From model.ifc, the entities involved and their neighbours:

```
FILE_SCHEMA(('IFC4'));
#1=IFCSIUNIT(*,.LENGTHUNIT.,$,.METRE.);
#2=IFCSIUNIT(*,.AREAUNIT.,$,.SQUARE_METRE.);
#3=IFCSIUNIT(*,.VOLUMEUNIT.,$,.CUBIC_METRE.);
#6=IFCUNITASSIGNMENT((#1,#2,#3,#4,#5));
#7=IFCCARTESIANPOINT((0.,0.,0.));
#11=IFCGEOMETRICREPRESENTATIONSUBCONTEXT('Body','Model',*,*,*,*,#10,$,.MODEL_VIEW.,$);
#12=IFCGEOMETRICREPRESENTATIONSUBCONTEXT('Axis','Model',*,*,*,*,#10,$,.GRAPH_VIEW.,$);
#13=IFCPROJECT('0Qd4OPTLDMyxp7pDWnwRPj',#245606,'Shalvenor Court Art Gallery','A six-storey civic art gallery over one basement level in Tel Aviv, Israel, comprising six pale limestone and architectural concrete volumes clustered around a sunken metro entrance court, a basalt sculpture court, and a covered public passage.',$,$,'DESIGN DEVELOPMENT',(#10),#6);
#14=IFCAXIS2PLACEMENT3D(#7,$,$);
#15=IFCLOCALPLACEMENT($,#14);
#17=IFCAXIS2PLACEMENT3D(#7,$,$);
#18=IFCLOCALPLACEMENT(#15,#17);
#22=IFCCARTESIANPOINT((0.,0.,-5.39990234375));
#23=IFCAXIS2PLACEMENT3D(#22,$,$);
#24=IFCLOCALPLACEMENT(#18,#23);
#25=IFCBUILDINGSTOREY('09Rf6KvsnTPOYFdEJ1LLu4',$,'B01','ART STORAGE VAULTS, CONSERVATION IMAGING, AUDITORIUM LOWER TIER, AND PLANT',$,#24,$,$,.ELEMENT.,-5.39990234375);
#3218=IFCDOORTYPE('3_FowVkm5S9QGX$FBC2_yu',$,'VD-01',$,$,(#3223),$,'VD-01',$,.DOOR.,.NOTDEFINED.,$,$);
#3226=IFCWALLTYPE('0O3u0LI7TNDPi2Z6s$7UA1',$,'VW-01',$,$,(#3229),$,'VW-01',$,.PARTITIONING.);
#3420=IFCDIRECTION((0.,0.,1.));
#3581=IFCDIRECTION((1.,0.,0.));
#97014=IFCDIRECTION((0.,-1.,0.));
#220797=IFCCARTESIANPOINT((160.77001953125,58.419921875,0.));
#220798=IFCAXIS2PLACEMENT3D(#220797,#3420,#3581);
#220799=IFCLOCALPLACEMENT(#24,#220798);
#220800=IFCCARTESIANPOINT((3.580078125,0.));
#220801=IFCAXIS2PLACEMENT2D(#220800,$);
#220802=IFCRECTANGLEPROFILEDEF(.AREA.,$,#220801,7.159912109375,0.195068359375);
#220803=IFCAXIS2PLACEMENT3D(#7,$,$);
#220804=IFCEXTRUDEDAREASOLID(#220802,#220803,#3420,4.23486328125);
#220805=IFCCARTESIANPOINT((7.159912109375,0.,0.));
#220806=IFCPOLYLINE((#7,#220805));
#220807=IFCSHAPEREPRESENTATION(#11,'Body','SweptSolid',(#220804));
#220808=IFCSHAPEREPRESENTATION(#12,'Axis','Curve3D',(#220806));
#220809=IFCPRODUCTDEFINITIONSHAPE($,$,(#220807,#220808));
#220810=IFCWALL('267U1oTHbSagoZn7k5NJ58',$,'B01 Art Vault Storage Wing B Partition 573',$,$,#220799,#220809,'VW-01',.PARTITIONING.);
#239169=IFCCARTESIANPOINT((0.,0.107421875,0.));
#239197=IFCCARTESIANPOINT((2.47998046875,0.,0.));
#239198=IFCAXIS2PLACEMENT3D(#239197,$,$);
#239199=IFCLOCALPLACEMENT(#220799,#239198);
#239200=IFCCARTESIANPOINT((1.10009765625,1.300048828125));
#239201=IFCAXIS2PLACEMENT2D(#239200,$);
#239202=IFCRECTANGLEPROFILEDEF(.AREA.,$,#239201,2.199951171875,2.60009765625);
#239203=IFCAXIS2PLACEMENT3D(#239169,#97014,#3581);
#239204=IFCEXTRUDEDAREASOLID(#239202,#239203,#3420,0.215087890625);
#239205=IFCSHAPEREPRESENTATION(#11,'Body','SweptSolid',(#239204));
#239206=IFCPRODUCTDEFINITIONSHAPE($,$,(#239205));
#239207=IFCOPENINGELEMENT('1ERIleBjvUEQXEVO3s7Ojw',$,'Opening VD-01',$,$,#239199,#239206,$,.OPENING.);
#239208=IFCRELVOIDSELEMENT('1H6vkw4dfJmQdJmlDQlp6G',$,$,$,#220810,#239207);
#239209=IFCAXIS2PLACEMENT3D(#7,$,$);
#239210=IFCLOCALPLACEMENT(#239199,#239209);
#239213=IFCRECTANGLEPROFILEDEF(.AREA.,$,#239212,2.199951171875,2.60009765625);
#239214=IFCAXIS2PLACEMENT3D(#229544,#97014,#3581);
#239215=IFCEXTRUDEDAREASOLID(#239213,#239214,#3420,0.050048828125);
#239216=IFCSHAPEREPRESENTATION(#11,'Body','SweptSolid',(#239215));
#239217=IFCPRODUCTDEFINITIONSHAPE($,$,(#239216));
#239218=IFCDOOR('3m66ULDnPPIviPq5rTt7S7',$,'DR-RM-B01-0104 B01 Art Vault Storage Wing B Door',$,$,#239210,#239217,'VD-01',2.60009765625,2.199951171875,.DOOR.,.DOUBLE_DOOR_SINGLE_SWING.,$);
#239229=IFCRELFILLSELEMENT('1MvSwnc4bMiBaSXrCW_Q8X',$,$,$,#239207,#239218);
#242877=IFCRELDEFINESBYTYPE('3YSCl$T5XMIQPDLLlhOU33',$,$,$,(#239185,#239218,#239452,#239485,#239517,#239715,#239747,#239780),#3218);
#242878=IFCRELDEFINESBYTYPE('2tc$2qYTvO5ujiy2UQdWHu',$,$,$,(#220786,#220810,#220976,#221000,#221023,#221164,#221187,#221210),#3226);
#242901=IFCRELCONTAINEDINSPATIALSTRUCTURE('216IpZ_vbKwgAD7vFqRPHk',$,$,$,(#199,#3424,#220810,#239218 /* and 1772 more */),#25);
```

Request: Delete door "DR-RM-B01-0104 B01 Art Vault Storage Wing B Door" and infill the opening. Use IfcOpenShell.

```python
import ifcopenshell
import ifcopenshell.api.feature
import ifcopenshell.api.root
import ifcopenshell.geom
import ifcopenshell.util.shape

model = ifcopenshell.open("model.ifc")
settings = ifcopenshell.geom.settings()


def volume(element):
    """Net volume in cubic metres, openings subtracted."""
    shape = ifcopenshell.geom.create_shape(settings, element)
    return ifcopenshell.util.shape.get_volume(shape.geometry)


door = model.by_guid("3m66ULDnPPIviPq5rTt7S7")
opening = door.FillsVoids[0].RelatingOpeningElement
wall = opening.VoidsElements[0].RelatingBuildingElement
before = volume(wall)

ifcopenshell.api.root.remove_product(model, product=door)
ifcopenshell.api.feature.remove_feature(model, feature=opening)

after = volume(wall)

print(f"wall volume {before:.3f} -> {after:.3f} m3")

model.write("model_rev.ifc")
```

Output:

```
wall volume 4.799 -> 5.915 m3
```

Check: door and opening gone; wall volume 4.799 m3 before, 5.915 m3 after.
